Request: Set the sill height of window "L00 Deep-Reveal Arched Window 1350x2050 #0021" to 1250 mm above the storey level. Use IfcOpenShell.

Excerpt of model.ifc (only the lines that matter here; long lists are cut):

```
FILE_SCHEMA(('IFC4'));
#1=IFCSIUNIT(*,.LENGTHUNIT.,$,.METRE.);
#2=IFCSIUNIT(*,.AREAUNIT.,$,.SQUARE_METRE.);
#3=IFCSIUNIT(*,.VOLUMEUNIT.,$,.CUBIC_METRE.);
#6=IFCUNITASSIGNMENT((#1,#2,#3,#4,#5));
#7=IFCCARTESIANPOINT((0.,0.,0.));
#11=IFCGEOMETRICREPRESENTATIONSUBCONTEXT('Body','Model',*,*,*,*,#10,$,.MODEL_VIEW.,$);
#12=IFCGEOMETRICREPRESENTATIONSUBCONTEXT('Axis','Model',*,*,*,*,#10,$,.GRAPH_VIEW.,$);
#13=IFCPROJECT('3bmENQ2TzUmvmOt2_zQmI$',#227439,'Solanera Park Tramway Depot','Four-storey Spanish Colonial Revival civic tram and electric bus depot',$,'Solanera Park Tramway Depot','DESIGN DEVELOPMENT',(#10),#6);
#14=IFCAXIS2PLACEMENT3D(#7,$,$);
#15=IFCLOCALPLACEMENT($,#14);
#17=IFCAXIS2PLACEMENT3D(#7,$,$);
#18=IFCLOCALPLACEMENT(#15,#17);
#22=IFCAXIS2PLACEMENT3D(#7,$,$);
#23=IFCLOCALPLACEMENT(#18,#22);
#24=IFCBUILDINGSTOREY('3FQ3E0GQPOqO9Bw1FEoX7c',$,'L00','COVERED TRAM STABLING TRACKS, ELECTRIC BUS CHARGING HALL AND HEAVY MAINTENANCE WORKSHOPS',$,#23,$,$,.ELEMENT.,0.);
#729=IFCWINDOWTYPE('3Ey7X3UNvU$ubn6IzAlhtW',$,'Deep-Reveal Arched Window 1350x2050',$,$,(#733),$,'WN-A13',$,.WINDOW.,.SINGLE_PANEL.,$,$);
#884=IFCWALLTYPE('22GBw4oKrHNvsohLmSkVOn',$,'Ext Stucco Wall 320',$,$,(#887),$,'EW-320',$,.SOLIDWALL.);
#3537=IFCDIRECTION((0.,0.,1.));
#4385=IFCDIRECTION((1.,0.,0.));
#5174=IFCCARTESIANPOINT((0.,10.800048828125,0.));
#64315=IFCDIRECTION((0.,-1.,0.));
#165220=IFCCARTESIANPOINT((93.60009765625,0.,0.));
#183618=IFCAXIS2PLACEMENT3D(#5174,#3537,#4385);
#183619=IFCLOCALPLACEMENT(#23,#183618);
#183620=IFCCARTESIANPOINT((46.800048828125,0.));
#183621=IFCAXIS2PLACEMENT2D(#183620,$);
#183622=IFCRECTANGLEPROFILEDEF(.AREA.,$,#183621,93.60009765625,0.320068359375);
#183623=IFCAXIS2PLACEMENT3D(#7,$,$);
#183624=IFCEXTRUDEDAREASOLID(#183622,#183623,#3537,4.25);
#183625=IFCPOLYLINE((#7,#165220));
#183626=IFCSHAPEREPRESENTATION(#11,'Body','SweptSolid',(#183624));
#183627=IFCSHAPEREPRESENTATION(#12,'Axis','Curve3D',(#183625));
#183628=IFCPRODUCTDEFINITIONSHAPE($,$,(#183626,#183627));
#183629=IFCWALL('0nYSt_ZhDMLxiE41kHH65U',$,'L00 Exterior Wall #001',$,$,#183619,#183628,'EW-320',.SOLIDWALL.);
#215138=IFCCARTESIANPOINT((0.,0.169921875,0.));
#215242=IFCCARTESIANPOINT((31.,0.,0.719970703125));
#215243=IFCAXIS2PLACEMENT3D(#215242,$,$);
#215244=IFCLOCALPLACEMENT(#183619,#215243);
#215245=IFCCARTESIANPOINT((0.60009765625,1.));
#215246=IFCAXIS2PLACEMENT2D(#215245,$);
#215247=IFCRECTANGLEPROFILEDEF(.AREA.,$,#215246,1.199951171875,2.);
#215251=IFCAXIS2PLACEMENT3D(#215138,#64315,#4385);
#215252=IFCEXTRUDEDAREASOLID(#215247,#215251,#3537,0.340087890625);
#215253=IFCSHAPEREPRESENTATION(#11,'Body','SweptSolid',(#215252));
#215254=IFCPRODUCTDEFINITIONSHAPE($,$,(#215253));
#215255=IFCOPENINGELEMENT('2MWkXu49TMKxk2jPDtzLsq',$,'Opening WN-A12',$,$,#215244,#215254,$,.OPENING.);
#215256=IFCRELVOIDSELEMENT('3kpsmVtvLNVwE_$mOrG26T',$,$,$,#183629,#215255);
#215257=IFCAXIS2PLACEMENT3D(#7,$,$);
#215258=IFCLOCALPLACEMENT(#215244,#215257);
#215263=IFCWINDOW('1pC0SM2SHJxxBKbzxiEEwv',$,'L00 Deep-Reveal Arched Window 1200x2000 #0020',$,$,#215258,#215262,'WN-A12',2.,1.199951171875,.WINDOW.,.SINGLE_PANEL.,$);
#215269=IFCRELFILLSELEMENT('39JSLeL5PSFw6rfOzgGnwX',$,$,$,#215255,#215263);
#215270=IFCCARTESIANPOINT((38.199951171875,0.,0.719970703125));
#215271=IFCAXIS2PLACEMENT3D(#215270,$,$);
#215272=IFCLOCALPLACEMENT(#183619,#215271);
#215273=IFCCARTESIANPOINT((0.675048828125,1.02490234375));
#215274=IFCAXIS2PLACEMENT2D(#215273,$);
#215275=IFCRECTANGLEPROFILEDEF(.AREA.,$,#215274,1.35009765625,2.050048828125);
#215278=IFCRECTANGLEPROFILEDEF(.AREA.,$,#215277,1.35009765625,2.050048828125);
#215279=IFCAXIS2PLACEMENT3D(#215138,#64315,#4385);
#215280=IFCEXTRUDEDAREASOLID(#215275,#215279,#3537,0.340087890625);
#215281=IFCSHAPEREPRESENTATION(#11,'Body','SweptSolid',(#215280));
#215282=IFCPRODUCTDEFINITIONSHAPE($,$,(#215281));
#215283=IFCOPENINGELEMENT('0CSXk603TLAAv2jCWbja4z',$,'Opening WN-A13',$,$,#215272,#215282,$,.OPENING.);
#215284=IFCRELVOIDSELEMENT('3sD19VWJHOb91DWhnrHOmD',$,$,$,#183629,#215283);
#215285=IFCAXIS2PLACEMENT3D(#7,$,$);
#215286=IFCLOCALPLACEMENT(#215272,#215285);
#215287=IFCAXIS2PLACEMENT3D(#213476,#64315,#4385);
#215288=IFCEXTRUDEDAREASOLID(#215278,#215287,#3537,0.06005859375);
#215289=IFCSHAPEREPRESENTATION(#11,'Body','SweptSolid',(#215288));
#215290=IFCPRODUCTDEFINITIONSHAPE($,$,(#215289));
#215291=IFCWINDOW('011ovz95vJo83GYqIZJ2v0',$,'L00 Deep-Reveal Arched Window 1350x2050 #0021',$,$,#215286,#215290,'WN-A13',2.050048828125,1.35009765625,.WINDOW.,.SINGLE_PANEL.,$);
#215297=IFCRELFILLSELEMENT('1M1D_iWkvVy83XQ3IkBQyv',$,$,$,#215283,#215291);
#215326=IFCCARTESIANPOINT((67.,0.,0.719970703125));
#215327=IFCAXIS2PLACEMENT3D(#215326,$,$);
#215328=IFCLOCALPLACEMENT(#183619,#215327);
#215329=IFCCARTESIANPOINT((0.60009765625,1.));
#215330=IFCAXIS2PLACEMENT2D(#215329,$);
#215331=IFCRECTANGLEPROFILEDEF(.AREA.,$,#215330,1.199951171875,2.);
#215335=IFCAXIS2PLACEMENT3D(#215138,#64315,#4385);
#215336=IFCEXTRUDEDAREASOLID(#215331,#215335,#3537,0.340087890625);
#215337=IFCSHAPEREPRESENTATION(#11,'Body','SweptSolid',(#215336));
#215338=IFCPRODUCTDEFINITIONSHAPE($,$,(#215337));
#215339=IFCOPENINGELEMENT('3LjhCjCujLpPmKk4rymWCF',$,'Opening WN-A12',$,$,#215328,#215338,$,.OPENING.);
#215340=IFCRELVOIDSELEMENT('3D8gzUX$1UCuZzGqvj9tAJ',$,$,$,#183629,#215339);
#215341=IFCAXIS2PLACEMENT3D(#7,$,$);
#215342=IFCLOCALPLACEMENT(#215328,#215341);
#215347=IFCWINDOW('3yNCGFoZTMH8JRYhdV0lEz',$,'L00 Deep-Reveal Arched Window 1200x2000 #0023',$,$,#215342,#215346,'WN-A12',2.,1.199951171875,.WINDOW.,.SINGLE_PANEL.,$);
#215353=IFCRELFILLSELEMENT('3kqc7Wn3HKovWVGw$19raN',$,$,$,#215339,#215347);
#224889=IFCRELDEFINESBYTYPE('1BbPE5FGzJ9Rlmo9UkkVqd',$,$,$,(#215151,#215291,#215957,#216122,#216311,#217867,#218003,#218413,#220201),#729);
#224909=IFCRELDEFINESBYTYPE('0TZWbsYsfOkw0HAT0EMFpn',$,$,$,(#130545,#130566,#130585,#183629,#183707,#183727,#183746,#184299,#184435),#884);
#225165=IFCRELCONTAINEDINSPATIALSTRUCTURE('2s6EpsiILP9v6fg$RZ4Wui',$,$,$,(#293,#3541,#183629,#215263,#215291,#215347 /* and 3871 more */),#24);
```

```python
import numpy as np
import ifcopenshell
import ifcopenshell.api.geometry
import ifcopenshell.geom
import ifcopenshell.util.element
import ifcopenshell.util.placement
import ifcopenshell.util.shape
import ifcopenshell.util.unit

model = ifcopenshell.open("model.ifc")
unit_scale = ifcopenshell.util.unit.calculate_unit_scale(model)

window = model.by_id(215291)
opening = window.FillsVoids[0].RelatingOpeningElement
storey = ifcopenshell.util.element.get_container(window, ifc_class="IfcBuildingStorey")
level = ifcopenshell.util.placement.get_local_placement(storey.ObjectPlacement)[2, 3]

# The opening's origin need not be at the sill, so measure its lowest point.
shape = ifcopenshell.geom.create_shape(ifcopenshell.geom.settings(), opening)
bottom = ifcopenshell.util.shape.get_shape_bottom_elevation(shape, shape.geometry) / unit_scale
dz = level + 1.25 / unit_scale - bottom

shift = np.array([0.0, 0.0, dz])
# The window is placed relative to its opening, so it follows when the opening moves.
matrix = ifcopenshell.util.placement.get_local_placement(opening.ObjectPlacement)
matrix[:3, 3] += shift
ifcopenshell.api.geometry.edit_object_placement(
    model, product=opening, matrix=matrix, is_si=False, should_transform_children=True
)

print(f"moved by {dz * unit_scale:+.3f} m")

model.write("model_edited.ifc")
```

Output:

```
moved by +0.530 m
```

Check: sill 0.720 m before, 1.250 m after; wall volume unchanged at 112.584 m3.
